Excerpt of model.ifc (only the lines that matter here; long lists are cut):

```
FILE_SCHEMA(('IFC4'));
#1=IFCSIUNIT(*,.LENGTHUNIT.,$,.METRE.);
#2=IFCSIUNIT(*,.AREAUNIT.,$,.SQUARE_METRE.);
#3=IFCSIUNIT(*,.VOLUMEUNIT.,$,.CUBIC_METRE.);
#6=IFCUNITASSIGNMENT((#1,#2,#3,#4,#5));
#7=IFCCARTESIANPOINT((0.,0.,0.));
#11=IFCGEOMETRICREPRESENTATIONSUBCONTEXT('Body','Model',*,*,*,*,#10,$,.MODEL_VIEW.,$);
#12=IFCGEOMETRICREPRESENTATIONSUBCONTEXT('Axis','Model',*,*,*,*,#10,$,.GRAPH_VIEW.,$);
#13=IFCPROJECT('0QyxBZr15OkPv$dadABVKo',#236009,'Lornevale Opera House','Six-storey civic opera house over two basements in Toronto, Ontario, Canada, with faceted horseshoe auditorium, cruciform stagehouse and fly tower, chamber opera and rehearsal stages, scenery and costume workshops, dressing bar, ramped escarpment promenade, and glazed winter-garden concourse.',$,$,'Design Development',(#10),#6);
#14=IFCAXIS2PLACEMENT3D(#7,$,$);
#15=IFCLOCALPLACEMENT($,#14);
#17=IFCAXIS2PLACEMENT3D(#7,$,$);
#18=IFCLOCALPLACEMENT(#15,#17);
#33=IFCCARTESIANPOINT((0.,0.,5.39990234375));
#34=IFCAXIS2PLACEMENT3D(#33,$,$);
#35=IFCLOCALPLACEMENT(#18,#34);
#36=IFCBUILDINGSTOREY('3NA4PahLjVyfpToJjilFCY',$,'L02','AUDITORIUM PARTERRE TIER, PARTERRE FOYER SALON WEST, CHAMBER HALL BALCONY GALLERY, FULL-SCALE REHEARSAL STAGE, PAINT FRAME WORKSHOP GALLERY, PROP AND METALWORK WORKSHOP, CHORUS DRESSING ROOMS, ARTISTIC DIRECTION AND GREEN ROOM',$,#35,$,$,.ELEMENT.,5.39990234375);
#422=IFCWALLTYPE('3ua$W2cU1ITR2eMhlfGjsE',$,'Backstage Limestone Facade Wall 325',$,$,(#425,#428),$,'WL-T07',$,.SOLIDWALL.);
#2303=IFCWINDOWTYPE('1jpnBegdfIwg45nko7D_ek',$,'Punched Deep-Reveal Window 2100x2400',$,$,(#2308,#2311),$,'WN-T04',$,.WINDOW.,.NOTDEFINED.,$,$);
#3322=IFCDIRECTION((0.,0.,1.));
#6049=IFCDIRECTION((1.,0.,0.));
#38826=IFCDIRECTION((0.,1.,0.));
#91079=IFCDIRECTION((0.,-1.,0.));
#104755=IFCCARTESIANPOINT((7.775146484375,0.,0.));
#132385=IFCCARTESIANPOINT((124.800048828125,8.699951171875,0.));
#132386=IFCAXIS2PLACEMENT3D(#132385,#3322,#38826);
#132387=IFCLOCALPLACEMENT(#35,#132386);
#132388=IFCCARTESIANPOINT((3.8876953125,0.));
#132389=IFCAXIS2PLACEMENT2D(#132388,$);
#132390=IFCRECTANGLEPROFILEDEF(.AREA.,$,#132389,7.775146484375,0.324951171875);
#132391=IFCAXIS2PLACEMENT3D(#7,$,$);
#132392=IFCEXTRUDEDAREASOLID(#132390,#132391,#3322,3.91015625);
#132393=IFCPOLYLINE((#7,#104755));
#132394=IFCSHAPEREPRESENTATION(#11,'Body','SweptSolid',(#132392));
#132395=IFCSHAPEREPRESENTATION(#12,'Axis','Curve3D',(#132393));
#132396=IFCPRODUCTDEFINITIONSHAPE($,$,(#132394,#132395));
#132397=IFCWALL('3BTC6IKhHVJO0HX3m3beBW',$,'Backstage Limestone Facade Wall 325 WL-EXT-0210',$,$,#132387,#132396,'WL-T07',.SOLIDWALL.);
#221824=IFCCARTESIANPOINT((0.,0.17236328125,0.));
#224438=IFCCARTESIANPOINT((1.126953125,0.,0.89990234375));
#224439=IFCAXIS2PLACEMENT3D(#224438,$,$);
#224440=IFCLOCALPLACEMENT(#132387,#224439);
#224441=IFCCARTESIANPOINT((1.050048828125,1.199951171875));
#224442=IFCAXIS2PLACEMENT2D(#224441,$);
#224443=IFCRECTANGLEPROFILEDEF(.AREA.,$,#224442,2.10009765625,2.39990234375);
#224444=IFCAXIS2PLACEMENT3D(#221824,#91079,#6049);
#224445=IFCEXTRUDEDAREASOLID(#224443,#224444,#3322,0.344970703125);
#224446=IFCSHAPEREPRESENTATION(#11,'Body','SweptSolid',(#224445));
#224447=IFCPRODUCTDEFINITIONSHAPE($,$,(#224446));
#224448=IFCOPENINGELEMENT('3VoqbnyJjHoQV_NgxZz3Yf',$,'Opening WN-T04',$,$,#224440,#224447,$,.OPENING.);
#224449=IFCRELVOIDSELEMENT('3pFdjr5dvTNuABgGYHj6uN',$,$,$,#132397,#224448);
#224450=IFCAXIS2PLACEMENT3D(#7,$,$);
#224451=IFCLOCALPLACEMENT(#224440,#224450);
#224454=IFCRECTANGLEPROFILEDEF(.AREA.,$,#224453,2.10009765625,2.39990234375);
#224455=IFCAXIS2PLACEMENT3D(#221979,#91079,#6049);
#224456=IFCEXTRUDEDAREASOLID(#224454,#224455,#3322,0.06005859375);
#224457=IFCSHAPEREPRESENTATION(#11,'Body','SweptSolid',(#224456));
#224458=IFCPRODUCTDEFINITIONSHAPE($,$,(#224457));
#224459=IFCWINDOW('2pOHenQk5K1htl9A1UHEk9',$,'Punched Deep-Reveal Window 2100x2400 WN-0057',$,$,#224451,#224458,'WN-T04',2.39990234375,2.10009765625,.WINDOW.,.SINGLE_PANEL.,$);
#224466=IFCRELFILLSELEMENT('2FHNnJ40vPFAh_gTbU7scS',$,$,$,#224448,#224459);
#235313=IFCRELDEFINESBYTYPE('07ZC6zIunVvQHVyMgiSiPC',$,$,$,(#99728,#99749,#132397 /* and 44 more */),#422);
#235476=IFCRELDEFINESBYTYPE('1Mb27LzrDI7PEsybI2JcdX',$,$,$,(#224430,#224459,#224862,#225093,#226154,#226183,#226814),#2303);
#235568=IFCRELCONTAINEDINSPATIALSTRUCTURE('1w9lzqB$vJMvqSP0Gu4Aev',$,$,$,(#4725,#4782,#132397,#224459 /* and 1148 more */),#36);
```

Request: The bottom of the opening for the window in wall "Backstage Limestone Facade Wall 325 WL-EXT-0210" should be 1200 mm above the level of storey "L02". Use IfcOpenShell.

```python
import numpy as np
import ifcopenshell
import ifcopenshell.api.geometry
import ifcopenshell.geom
import ifcopenshell.util.element
import ifcopenshell.util.placement
import ifcopenshell.util.shape
import ifcopenshell.util.unit

model = ifcopenshell.open("model.ifc")
unit_scale = ifcopenshell.util.unit.calculate_unit_scale(model)

window = model.by_id(224459)
opening = window.FillsVoids[0].RelatingOpeningElement
storey = ifcopenshell.util.element.get_container(window, ifc_class="IfcBuildingStorey")
level = ifcopenshell.util.placement.get_local_placement(storey.ObjectPlacement)[2, 3]

# The opening's origin need not be at the sill, so measure its lowest point.
shape = ifcopenshell.geom.create_shape(ifcopenshell.geom.settings(), opening)
bottom = ifcopenshell.util.shape.get_shape_bottom_elevation(shape, shape.geometry) / unit_scale
dz = level + 1.2 - bottom

shift = np.array([0.0, 0.0, dz])
# The window is placed relative to its opening, so it follows when the opening moves.
matrix = ifcopenshell.util.placement.get_local_placement(opening.ObjectPlacement)
matrix[:3, 3] += shift
ifcopenshell.api.geometry.edit_object_placement(
    model, product=opening, matrix=matrix, is_si=False, should_transform_children=True
)

print(f"moved by {dz * unit_scale:+.3f} m")

model.write("model-out.ifc")
```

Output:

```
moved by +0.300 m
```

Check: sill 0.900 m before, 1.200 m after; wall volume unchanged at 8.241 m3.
